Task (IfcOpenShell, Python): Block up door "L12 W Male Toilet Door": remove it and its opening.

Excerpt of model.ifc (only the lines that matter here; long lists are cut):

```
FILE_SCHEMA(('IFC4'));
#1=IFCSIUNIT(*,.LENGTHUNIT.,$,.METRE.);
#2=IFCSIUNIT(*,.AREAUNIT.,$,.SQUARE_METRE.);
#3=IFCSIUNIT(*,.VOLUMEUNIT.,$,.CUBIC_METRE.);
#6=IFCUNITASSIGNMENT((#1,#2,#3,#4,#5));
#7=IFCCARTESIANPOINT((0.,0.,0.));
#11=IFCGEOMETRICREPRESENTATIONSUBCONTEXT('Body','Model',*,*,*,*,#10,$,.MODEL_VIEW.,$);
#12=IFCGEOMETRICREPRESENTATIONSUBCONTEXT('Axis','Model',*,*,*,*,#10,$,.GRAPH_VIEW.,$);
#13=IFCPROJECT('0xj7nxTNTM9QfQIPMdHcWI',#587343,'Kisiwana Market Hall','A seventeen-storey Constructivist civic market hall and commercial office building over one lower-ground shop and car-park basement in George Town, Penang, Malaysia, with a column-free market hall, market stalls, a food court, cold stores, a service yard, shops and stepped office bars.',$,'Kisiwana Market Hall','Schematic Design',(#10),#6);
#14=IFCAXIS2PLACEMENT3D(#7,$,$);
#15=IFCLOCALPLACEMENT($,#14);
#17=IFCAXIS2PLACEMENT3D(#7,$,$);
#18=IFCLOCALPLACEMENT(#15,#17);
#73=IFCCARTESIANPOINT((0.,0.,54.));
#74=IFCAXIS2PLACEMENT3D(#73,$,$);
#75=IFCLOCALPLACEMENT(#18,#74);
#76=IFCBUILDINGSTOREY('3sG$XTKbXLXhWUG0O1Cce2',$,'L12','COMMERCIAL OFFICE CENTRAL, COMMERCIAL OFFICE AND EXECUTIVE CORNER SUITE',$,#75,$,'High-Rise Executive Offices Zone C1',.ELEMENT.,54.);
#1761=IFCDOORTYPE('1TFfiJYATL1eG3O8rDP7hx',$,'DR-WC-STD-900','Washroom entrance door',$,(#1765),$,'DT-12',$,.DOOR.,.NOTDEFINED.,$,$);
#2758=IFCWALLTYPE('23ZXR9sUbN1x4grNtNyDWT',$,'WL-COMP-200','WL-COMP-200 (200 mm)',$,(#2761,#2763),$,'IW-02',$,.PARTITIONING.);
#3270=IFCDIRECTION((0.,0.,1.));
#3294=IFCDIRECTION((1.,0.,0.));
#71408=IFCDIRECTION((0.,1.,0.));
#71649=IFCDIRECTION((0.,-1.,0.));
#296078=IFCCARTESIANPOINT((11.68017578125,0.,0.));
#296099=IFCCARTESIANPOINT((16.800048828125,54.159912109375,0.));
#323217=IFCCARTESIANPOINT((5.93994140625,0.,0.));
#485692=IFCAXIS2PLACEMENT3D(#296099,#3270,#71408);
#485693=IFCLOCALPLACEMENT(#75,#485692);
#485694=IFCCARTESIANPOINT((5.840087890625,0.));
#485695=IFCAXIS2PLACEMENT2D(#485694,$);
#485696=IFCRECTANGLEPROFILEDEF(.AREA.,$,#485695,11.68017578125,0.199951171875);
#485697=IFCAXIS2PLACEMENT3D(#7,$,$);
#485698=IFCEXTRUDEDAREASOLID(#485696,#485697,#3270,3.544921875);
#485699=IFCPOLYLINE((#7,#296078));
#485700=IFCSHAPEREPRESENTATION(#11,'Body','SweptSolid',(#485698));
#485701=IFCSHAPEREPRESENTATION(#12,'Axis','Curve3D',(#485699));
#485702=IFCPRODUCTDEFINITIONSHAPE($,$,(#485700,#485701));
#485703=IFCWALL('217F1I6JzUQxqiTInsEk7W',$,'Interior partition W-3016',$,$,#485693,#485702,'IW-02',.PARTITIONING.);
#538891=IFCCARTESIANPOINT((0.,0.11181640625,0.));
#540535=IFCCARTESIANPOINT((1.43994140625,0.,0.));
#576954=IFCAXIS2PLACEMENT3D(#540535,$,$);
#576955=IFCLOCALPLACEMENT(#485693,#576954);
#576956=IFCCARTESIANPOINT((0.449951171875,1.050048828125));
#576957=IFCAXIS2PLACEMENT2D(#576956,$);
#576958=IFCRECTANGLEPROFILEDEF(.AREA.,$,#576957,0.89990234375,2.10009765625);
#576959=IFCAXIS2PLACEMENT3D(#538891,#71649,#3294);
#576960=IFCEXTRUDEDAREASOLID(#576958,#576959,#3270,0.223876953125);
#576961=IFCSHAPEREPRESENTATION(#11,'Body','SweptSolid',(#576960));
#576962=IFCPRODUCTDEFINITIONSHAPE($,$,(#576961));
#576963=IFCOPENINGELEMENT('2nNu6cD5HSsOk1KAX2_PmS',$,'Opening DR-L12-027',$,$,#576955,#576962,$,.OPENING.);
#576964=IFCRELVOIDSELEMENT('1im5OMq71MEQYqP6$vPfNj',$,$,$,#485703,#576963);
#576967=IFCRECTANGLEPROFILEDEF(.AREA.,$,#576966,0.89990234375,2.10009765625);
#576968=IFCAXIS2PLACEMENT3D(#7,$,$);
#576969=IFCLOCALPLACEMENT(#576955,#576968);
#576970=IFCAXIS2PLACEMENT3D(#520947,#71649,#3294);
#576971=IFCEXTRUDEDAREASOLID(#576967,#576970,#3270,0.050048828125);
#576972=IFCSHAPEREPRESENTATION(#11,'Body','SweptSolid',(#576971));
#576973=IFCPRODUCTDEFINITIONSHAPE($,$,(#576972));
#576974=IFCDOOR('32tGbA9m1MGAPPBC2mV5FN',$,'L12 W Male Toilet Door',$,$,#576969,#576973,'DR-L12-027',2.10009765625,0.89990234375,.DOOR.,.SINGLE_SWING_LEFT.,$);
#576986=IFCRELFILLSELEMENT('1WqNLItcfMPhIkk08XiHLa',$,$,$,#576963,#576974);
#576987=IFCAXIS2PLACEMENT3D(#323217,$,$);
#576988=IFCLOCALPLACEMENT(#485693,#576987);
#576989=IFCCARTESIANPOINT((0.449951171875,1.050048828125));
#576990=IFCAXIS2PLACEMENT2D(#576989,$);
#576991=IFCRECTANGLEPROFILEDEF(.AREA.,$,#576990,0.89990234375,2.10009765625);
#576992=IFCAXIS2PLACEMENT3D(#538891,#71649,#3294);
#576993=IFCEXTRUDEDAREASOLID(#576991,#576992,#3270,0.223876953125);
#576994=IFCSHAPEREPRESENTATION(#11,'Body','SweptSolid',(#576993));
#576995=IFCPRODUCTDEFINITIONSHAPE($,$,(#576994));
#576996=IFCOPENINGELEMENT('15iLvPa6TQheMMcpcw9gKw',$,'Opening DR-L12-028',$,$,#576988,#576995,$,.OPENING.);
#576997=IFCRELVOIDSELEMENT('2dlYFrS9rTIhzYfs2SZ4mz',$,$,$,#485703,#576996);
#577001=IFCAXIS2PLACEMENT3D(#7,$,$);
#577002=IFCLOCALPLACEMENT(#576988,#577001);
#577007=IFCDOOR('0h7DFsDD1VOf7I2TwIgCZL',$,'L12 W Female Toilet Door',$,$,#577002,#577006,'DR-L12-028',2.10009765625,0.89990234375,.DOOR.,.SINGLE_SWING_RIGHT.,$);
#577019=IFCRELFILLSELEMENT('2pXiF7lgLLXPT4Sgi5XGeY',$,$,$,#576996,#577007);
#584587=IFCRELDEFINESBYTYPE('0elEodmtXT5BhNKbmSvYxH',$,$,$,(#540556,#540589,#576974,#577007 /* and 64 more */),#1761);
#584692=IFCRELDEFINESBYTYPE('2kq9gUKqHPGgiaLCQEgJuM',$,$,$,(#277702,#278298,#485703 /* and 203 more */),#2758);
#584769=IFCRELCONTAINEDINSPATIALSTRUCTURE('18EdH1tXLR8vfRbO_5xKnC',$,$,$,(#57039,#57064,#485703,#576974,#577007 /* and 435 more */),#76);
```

```python
import ifcopenshell
import ifcopenshell.api.feature
import ifcopenshell.api.root
import ifcopenshell.geom
import ifcopenshell.util.shape

model = ifcopenshell.open("model.ifc")
settings = ifcopenshell.geom.settings()


def volume(element):
    """Net volume in cubic metres, openings subtracted."""
    shape = ifcopenshell.geom.create_shape(settings, element)
    return ifcopenshell.util.shape.get_volume(shape.geometry)


door = model.by_id(576974)
opening = door.FillsVoids[0].RelatingOpeningElement
wall = opening.VoidsElements[0].RelatingBuildingElement
before = volume(wall)

ifcopenshell.api.root.remove_product(model, product=door)
ifcopenshell.api.feature.remove_feature(model, feature=opening)

after = volume(wall)

print(f"wall volume {before:.3f} -> {after:.3f} m3")

model.write("model_edited.ifc")
```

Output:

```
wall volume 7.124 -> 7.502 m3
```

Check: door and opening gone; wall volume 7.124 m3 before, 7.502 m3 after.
